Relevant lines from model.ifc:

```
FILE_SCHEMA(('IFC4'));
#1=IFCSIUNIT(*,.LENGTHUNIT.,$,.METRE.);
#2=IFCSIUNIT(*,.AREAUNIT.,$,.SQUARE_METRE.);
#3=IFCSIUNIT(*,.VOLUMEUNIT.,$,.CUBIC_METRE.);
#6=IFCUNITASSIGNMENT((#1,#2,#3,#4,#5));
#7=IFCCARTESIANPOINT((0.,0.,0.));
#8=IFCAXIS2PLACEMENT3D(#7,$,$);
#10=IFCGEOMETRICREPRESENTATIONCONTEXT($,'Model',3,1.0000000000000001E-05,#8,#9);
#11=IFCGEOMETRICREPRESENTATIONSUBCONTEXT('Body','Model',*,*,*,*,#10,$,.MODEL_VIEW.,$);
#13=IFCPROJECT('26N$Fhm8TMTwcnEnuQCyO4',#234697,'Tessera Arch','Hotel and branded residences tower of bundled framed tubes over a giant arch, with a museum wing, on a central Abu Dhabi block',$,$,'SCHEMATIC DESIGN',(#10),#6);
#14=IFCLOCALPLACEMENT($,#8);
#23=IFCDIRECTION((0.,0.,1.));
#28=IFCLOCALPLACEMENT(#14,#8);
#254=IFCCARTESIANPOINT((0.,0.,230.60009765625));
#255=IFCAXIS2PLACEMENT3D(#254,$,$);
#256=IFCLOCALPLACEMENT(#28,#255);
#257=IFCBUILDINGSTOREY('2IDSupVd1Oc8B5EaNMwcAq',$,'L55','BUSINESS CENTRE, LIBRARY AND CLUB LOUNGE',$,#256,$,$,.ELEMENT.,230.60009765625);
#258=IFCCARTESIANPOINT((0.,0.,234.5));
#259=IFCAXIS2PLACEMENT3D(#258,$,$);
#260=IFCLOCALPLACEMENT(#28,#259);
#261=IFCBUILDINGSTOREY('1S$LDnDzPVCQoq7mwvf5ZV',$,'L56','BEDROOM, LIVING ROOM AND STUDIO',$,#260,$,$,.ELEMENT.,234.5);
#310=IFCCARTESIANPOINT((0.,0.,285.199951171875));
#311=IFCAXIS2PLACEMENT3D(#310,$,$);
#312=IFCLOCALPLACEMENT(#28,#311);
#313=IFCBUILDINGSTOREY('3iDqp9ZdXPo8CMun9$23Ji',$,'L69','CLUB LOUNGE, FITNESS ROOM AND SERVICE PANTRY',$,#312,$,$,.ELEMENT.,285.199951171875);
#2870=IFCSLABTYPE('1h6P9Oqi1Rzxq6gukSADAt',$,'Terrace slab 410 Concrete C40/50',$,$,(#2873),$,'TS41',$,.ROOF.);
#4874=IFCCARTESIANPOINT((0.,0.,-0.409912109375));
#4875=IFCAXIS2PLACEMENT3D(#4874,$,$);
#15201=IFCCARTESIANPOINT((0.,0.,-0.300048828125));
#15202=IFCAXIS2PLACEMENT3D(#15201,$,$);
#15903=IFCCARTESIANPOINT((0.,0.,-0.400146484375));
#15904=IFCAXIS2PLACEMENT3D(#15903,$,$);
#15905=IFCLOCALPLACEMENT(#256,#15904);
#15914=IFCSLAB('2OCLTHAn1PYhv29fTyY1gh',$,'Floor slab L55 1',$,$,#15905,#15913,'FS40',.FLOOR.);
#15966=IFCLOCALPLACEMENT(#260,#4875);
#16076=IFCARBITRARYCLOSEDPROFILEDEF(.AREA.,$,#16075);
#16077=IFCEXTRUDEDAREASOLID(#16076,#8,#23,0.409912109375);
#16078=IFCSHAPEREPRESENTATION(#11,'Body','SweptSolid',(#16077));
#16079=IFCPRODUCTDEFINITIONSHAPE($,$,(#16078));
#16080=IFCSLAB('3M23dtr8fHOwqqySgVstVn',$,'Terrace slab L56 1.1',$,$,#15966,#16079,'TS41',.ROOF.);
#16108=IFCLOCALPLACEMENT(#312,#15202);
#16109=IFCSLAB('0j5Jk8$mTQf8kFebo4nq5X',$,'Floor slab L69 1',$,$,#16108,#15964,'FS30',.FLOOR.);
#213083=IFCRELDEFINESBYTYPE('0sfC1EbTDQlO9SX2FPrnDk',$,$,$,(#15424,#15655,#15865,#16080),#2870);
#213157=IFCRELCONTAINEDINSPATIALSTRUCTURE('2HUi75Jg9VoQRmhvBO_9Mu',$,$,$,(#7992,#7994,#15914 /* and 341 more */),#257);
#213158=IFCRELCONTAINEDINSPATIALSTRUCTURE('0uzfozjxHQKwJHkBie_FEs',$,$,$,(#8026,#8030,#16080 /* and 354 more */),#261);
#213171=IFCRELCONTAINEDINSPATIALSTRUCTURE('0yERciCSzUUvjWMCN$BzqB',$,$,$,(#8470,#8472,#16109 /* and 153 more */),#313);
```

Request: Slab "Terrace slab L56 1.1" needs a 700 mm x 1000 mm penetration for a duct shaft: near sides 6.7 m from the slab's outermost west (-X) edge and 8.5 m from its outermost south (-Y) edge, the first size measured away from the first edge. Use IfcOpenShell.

```python
import numpy as np
import ifcopenshell
import ifcopenshell.api.feature
import ifcopenshell.api.geometry
import ifcopenshell.api.root
import ifcopenshell.geom
import ifcopenshell.util.placement
import ifcopenshell.util.representation
import ifcopenshell.util.shape
import ifcopenshell.util.unit

model = ifcopenshell.open("model.ifc")
unit_scale = ifcopenshell.util.unit.calculate_unit_scale(model)
settings = ifcopenshell.geom.settings()


def volume(element):
    """Net volume in cubic metres, openings subtracted."""
    shape = ifcopenshell.geom.create_shape(settings, element)
    return ifcopenshell.util.shape.get_volume(shape.geometry)


slab = model.by_guid("3M23dtr8fHOwqqySgVstVn")
before = volume(slab)

# Extent in the slab's own axes, in metres. The edges named are its -X and -Y sides.
slab_shape = ifcopenshell.geom.create_shape(settings, slab)
vertices = ifcopenshell.util.shape.get_vertices(slab_shape.geometry)
x_min, y_min, bottom = vertices.min(axis=0)
top = vertices[:, 2].max()

opening = ifcopenshell.api.root.create_entity(model, ifc_class="IfcOpeningElement", name="Duct shaft opening", predefined_type="OPENING")
context = ifcopenshell.util.representation.get_context(model, "Model", "Body", "MODEL_VIEW")
width, depth = 0.7, 1
outline = [(0.0, 0.0), (width, 0.0), (width, depth), (0.0, depth), (0.0, 0.0)]
# Overshoot both faces by 50 mm so the cut is clean.
shape = ifcopenshell.api.geometry.add_slab_representation(
    model, context=context, depth=top - bottom + 0.1, polyline=outline
)
ifcopenshell.api.geometry.assign_representation(model, product=opening, representation=shape)

matrix = ifcopenshell.util.placement.get_local_placement(slab.ObjectPlacement)
matrix[:, 3] = matrix @ np.append(np.array([x_min + 6.7, y_min + 8.5, bottom - 0.05]) / unit_scale, 1.0)
ifcopenshell.api.geometry.edit_object_placement(model, product=opening, matrix=matrix, is_si=False)
ifcopenshell.api.feature.add_feature(model, feature=opening, element=slab)

after = volume(slab)

print(f"slab volume {before:.3f} -> {after:.3f} m3")

model.write("model_updated.ifc")
```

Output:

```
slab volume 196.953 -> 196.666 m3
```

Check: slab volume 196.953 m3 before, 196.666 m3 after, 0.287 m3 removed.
